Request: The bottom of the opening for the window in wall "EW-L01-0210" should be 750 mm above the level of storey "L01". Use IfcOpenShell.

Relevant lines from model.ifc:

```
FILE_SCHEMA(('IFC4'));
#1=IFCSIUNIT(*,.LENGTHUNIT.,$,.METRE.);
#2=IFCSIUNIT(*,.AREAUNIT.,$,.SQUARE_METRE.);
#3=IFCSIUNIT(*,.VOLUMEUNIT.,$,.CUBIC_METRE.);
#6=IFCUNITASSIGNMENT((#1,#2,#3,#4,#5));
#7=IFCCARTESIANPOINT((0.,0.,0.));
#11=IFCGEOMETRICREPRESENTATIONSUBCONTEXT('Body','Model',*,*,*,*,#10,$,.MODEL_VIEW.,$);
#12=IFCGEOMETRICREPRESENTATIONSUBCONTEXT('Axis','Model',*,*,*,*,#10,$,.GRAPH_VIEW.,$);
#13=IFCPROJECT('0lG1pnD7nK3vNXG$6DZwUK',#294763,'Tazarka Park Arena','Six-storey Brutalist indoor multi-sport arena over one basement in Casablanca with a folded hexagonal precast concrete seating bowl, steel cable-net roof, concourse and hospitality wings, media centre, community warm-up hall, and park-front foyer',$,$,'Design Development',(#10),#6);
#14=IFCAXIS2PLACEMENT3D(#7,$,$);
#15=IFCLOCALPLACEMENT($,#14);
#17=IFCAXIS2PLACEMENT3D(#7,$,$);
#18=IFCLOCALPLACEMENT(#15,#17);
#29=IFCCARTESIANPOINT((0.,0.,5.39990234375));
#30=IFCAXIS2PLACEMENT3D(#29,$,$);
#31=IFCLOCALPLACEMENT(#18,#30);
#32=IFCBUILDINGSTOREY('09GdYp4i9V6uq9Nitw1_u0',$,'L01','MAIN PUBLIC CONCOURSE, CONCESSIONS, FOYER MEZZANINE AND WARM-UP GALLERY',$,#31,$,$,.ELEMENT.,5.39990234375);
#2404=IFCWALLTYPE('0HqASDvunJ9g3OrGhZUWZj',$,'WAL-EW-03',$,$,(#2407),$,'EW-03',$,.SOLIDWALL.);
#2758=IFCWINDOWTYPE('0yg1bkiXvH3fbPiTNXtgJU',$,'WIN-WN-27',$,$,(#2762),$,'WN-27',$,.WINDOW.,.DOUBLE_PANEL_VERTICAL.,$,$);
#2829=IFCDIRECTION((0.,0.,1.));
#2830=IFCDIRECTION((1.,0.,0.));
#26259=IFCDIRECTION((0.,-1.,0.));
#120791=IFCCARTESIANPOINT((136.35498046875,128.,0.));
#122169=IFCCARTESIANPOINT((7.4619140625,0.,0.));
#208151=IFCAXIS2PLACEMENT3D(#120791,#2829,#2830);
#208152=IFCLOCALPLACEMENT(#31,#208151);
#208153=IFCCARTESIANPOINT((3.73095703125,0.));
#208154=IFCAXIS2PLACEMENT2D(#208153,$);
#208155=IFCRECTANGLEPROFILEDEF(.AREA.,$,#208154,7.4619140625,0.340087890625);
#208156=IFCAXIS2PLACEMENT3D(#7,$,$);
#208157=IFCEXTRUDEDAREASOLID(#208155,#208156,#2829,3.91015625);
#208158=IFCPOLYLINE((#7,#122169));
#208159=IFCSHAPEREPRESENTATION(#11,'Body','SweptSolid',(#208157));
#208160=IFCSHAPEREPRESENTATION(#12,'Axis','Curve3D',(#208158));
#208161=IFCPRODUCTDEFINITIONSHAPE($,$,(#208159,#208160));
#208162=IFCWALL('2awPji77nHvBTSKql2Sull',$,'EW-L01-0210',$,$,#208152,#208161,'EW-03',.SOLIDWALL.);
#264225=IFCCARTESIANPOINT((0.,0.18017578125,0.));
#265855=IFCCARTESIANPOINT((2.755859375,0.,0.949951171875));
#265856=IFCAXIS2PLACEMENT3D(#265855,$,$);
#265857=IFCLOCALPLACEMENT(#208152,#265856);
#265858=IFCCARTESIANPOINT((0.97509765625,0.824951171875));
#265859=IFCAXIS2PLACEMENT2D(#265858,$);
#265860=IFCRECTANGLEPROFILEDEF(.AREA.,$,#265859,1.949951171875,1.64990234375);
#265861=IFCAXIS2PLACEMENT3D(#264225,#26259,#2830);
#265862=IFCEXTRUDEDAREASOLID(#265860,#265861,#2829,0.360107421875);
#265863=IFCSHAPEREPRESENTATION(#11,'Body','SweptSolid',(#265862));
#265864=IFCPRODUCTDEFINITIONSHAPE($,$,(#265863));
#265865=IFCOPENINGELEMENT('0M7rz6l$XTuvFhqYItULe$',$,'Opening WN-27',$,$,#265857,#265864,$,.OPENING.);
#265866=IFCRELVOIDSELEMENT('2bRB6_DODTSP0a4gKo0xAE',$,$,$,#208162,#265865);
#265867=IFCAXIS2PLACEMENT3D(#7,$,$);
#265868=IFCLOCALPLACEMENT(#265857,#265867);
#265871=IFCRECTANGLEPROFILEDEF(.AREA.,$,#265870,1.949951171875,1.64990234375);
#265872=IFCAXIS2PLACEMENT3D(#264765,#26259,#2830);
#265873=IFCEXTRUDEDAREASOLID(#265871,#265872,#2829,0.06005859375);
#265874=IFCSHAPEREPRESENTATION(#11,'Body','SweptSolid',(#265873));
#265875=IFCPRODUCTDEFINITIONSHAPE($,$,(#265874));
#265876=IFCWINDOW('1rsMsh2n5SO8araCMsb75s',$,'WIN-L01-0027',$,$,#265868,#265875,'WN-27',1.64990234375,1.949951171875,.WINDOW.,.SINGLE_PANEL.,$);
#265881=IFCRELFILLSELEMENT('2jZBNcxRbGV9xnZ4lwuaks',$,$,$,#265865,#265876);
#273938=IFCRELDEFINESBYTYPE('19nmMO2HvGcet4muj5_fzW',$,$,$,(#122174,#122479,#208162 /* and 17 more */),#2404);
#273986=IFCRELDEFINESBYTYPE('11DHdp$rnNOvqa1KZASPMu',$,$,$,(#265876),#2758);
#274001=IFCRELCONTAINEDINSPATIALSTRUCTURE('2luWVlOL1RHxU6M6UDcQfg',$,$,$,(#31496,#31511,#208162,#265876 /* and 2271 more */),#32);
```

```python
import numpy as np
import ifcopenshell
import ifcopenshell.api.geometry
import ifcopenshell.geom
import ifcopenshell.util.element
import ifcopenshell.util.placement
import ifcopenshell.util.shape
import ifcopenshell.util.unit

model = ifcopenshell.open("model.ifc")
unit_scale = ifcopenshell.util.unit.calculate_unit_scale(model)

window = model.by_guid("1rsMsh2n5SO8araCMsb75s")
opening = window.FillsVoids[0].RelatingOpeningElement
storey = ifcopenshell.util.element.get_container(window, ifc_class="IfcBuildingStorey")
level = ifcopenshell.util.placement.get_local_placement(storey.ObjectPlacement)[2, 3]

# The opening's origin need not be at the sill, so measure its lowest point.
shape = ifcopenshell.geom.create_shape(ifcopenshell.geom.settings(), opening)
bottom = ifcopenshell.util.shape.get_shape_bottom_elevation(shape, shape.geometry) / unit_scale
dz = level + 0.75 / unit_scale - bottom

shift = np.array([0.0, 0.0, dz])
# The window is placed relative to its opening, so it follows when the opening moves.
matrix = ifcopenshell.util.placement.get_local_placement(opening.ObjectPlacement)
matrix[:3, 3] += shift
ifcopenshell.api.geometry.edit_object_placement(
    model, product=opening, matrix=matrix, is_si=False, should_transform_children=True
)

print(f"moved by {dz * unit_scale:+.3f} m")

model.write("model_edited.ifc")
```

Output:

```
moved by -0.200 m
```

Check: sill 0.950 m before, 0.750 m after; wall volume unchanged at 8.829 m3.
